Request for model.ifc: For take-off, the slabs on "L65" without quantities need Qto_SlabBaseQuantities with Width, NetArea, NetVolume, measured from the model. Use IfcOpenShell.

First a look at what the model holds.

```python
import ifcopenshell
import ifcopenshell.util.element
import ifcopenshell.util.unit

model = ifcopenshell.open("model.ifc")
print(model.schema)
for unit_type in ("LENGTHUNIT", "AREAUNIT", "VOLUMEUNIT"):
    print(unit_type, ifcopenshell.util.unit.calculate_unit_scale(model, unit_type))
storey = next(s for s in model.by_type("IfcBuildingStorey") if s.Name == "L65")
slabs = [e for e in ifcopenshell.util.element.get_decomposition(storey) if e.is_a("IfcSlab")]
for e in sorted(slabs, key=lambda e: e.id()):
    print(e.id(), e.is_a(), e.Name, list(ifcopenshell.util.element.get_psets(e, qtos_only=True)), sep=" | ")
```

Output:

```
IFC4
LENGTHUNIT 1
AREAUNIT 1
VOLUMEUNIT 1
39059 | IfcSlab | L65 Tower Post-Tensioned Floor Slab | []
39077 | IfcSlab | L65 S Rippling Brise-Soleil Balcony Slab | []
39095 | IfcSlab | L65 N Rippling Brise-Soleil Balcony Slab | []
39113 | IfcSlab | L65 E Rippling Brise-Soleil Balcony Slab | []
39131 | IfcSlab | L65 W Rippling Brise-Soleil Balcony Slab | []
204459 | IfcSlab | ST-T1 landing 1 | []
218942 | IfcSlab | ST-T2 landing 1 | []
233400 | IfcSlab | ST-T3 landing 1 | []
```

```python
import ifcopenshell
import ifcopenshell.api.pset
import ifcopenshell.geom
import ifcopenshell.util.element
import ifcopenshell.util.shape
import ifcopenshell.util.unit

model = ifcopenshell.open("model.ifc")
unit_scale = ifcopenshell.util.unit.calculate_unit_scale(model)
area_scale = ifcopenshell.util.unit.calculate_unit_scale(model, "AREAUNIT")
volume_scale = ifcopenshell.util.unit.calculate_unit_scale(model, "VOLUMEUNIT")
settings = ifcopenshell.geom.settings()

storey = next(s for s in model.by_type("IfcBuildingStorey") if s.Name == "L65")
slabs = [e for e in ifcopenshell.util.element.get_decomposition(storey) if e.is_a("IfcSlab")]

for e in sorted(slabs, key=lambda e: e.id()):
    if ifcopenshell.util.element.get_psets(e, qtos_only=True, should_inherit=False):
        continue
    # Geometry comes back in metres, in the element's own axes.
    shape = ifcopenshell.geom.create_shape(settings, e)
    values = {
        "Width": ifcopenshell.util.shape.get_z(shape.geometry) / unit_scale,
        "NetArea": ifcopenshell.util.shape.get_footprint_area(shape.geometry) / area_scale,
        "NetVolume": ifcopenshell.util.shape.get_volume(shape.geometry) / volume_scale,
    }
    qto = ifcopenshell.api.pset.add_qto(model, product=e, name="Qto_SlabBaseQuantities")
    ifcopenshell.api.pset.edit_qto(model, qto=qto, properties=values)
    print(e.id(), {k: round(v, 3) for k, v in values.items()})

model.write("model_updated.ifc")
```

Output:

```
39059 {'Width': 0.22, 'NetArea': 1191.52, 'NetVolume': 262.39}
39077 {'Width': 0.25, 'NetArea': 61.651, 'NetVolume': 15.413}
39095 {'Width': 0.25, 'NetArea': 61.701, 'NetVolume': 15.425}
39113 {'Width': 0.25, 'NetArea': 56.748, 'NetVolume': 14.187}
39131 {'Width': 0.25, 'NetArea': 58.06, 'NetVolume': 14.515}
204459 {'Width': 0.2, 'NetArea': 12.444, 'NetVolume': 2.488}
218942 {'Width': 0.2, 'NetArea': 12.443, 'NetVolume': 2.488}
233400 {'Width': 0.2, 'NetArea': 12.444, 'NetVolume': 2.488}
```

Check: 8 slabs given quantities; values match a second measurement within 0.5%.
